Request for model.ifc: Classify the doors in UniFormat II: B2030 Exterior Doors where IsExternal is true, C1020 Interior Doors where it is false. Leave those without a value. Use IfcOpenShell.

First a look at what the model holds.

```python
import ifcopenshell
import ifcopenshell.util.element

model = ifcopenshell.open("model.ifc")
print(model.schema)
print("classifications:", [c.Name for c in model.by_type("IfcClassification")])
values = [ifcopenshell.util.element.get_pset(e, "Pset_DoorCommon", "IsExternal") for e in model.by_type("IfcDoor")]
for value in (True, False, None):
    print("IsExternal", value, values.count(value))
```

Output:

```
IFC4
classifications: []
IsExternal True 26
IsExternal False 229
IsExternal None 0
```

```python
import ifcopenshell
import ifcopenshell.api.classification
import ifcopenshell.util.element

model = ifcopenshell.open("model.ifc")

system = ifcopenshell.api.classification.add_classification(model, classification="UniFormat II")

doors = model.by_type("IfcDoor")
external = {e: ifcopenshell.util.element.get_pset(e, "Pset_DoorCommon", "IsExternal") for e in doors}
for flag, code, name in ((True, "B2030", "Exterior Doors"), (False, "C1020", "Interior Doors")):
    products = [e for e in doors if external[e] is flag]
    ifcopenshell.api.classification.add_reference(
        model, products=products, classification=system, identification=code, name=name
    )
    print(code, len(products))

model.write("model_updated.ifc")
```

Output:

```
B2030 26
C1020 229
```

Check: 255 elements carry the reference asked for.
